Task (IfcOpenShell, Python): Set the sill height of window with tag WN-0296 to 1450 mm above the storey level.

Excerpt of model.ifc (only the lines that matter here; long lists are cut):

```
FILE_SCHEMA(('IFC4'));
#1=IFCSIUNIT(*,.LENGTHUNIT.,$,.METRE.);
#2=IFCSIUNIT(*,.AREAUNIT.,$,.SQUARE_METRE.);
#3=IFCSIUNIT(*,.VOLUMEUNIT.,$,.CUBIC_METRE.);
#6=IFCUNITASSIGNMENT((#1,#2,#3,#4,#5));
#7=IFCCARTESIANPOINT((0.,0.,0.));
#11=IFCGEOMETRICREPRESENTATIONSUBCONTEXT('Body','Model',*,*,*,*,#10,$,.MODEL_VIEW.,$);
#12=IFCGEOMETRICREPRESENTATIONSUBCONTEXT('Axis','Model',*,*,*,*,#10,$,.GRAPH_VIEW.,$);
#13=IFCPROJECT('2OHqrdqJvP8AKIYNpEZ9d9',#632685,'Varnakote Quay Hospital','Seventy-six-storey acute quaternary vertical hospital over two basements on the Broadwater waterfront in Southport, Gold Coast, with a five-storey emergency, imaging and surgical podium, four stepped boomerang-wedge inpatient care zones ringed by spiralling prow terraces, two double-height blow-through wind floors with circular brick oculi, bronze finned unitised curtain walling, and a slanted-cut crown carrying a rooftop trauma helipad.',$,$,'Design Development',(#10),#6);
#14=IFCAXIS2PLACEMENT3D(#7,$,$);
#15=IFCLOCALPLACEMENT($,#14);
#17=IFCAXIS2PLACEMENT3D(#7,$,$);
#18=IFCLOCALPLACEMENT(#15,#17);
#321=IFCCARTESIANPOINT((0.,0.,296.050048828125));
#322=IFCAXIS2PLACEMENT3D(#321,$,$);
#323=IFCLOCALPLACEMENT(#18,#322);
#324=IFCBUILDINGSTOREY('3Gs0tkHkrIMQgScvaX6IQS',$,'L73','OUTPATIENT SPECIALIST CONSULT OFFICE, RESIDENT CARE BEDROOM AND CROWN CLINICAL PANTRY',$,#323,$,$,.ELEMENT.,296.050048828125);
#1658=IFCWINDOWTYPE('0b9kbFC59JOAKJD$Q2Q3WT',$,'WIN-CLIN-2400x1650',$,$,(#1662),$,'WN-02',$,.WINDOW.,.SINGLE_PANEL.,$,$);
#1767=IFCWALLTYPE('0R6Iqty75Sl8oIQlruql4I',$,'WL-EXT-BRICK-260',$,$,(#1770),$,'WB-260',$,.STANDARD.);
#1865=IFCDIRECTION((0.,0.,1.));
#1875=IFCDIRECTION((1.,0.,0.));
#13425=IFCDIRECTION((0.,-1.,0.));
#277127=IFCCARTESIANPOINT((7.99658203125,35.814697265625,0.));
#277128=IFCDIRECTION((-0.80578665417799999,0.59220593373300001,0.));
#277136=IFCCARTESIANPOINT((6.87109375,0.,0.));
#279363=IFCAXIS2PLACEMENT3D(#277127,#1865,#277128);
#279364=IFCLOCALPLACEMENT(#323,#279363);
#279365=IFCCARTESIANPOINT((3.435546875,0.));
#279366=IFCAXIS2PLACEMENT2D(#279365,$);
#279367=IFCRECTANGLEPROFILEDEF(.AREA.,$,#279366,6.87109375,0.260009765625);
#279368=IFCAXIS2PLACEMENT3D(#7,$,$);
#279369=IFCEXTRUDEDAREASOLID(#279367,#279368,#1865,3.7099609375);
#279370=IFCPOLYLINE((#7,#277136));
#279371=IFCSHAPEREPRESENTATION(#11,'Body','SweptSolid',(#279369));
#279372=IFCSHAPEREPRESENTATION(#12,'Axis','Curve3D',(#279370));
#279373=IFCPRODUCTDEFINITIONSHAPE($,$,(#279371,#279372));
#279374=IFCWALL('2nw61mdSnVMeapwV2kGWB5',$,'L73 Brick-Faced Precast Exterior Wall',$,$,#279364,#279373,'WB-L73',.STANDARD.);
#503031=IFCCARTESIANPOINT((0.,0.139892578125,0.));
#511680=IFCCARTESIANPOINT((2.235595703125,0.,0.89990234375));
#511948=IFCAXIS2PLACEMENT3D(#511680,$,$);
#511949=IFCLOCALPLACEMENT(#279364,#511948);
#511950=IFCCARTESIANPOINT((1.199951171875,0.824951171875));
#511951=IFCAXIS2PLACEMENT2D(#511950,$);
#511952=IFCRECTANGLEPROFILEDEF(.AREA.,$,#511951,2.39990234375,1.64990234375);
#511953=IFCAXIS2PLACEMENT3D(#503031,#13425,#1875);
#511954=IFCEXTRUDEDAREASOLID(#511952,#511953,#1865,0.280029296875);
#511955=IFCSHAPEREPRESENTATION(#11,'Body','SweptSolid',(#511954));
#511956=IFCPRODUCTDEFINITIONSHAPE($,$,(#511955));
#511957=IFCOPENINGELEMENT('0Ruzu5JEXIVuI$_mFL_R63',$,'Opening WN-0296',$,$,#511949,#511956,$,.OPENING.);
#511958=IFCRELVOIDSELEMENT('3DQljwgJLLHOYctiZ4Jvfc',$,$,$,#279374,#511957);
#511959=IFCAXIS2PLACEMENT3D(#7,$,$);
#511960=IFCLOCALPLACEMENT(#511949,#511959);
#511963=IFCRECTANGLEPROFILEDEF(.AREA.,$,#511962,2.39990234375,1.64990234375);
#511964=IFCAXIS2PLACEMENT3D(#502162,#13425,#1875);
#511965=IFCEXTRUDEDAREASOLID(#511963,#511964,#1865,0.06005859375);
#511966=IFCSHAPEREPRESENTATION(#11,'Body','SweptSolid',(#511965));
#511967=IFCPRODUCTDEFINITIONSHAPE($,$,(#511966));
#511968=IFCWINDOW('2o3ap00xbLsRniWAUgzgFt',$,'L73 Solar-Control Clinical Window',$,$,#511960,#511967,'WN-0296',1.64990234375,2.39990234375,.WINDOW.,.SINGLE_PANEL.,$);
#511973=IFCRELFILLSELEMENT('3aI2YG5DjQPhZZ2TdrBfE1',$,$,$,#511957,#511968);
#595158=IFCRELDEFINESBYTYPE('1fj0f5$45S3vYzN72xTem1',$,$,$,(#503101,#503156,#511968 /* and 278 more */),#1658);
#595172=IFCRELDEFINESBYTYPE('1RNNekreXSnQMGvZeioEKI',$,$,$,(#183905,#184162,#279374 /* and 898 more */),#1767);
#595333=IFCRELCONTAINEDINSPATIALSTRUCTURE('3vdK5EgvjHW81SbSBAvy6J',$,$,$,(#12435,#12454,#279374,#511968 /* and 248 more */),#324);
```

```python
import numpy as np
import ifcopenshell
import ifcopenshell.api.geometry
import ifcopenshell.geom
import ifcopenshell.util.element
import ifcopenshell.util.placement
import ifcopenshell.util.shape
import ifcopenshell.util.unit

model = ifcopenshell.open("model.ifc")
unit_scale = ifcopenshell.util.unit.calculate_unit_scale(model)

window = model.by_guid("2o3ap00xbLsRniWAUgzgFt")
opening = window.FillsVoids[0].RelatingOpeningElement
storey = ifcopenshell.util.element.get_container(window, ifc_class="IfcBuildingStorey")
level = ifcopenshell.util.placement.get_local_placement(storey.ObjectPlacement)[2, 3]

# The opening's origin need not be at the sill, so measure its lowest point.
shape = ifcopenshell.geom.create_shape(ifcopenshell.geom.settings(), opening)
bottom = ifcopenshell.util.shape.get_shape_bottom_elevation(shape, shape.geometry) / unit_scale
dz = level + 1.45 / unit_scale - bottom

shift = np.array([0.0, 0.0, dz])
# The window is placed relative to its opening, so it follows when the opening moves.
matrix = ifcopenshell.util.placement.get_local_placement(opening.ObjectPlacement)
matrix[:3, 3] += shift
ifcopenshell.api.geometry.edit_object_placement(
    model, product=opening, matrix=matrix, is_si=False, should_transform_children=True
)

print(f"moved by {dz * unit_scale:+.3f} m")

model.write("model_v2.ifc")
```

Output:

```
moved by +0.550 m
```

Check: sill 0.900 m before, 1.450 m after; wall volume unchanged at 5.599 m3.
